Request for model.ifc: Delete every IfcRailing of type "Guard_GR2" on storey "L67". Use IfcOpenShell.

First a look at what the model holds.

```python
import ifcopenshell
import ifcopenshell.util.element

model = ifcopenshell.open("model.ifc")
print(model.schema)
storey = next(s for s in model.by_type("IfcBuildingStorey") if s.Name == "L67")
railings = [e for e in ifcopenshell.util.element.get_decomposition(storey) if e.is_a("IfcRailing")]
seen = {}
for e in railings:
    element_type = ifcopenshell.util.element.get_type(e)
    name = element_type.Name if element_type not in (None, e) else None
    seen[name] = seen.get(name, 0) + 1
for name, count in sorted(seen.items(), key=str):
    print(count, "x", name)
```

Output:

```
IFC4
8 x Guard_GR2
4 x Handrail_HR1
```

```python
import ifcopenshell
import ifcopenshell.api.root
import ifcopenshell.util.element

model = ifcopenshell.open("model.ifc")

storey = next(s for s in model.by_type("IfcBuildingStorey") if s.Name == "L67")
railings = [e for e in ifcopenshell.util.element.get_decomposition(storey) if e.is_a("IfcRailing")]
targets = [e for e in railings if (t := ifcopenshell.util.element.get_type(e)) not in (None, e) and t.Name == "Guard_GR2"]

for e in targets:
    ifcopenshell.api.root.remove_product(model, product=e)
print(len(targets), "removed")

model.write("model-out.ifc")
```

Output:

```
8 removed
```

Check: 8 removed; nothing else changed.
